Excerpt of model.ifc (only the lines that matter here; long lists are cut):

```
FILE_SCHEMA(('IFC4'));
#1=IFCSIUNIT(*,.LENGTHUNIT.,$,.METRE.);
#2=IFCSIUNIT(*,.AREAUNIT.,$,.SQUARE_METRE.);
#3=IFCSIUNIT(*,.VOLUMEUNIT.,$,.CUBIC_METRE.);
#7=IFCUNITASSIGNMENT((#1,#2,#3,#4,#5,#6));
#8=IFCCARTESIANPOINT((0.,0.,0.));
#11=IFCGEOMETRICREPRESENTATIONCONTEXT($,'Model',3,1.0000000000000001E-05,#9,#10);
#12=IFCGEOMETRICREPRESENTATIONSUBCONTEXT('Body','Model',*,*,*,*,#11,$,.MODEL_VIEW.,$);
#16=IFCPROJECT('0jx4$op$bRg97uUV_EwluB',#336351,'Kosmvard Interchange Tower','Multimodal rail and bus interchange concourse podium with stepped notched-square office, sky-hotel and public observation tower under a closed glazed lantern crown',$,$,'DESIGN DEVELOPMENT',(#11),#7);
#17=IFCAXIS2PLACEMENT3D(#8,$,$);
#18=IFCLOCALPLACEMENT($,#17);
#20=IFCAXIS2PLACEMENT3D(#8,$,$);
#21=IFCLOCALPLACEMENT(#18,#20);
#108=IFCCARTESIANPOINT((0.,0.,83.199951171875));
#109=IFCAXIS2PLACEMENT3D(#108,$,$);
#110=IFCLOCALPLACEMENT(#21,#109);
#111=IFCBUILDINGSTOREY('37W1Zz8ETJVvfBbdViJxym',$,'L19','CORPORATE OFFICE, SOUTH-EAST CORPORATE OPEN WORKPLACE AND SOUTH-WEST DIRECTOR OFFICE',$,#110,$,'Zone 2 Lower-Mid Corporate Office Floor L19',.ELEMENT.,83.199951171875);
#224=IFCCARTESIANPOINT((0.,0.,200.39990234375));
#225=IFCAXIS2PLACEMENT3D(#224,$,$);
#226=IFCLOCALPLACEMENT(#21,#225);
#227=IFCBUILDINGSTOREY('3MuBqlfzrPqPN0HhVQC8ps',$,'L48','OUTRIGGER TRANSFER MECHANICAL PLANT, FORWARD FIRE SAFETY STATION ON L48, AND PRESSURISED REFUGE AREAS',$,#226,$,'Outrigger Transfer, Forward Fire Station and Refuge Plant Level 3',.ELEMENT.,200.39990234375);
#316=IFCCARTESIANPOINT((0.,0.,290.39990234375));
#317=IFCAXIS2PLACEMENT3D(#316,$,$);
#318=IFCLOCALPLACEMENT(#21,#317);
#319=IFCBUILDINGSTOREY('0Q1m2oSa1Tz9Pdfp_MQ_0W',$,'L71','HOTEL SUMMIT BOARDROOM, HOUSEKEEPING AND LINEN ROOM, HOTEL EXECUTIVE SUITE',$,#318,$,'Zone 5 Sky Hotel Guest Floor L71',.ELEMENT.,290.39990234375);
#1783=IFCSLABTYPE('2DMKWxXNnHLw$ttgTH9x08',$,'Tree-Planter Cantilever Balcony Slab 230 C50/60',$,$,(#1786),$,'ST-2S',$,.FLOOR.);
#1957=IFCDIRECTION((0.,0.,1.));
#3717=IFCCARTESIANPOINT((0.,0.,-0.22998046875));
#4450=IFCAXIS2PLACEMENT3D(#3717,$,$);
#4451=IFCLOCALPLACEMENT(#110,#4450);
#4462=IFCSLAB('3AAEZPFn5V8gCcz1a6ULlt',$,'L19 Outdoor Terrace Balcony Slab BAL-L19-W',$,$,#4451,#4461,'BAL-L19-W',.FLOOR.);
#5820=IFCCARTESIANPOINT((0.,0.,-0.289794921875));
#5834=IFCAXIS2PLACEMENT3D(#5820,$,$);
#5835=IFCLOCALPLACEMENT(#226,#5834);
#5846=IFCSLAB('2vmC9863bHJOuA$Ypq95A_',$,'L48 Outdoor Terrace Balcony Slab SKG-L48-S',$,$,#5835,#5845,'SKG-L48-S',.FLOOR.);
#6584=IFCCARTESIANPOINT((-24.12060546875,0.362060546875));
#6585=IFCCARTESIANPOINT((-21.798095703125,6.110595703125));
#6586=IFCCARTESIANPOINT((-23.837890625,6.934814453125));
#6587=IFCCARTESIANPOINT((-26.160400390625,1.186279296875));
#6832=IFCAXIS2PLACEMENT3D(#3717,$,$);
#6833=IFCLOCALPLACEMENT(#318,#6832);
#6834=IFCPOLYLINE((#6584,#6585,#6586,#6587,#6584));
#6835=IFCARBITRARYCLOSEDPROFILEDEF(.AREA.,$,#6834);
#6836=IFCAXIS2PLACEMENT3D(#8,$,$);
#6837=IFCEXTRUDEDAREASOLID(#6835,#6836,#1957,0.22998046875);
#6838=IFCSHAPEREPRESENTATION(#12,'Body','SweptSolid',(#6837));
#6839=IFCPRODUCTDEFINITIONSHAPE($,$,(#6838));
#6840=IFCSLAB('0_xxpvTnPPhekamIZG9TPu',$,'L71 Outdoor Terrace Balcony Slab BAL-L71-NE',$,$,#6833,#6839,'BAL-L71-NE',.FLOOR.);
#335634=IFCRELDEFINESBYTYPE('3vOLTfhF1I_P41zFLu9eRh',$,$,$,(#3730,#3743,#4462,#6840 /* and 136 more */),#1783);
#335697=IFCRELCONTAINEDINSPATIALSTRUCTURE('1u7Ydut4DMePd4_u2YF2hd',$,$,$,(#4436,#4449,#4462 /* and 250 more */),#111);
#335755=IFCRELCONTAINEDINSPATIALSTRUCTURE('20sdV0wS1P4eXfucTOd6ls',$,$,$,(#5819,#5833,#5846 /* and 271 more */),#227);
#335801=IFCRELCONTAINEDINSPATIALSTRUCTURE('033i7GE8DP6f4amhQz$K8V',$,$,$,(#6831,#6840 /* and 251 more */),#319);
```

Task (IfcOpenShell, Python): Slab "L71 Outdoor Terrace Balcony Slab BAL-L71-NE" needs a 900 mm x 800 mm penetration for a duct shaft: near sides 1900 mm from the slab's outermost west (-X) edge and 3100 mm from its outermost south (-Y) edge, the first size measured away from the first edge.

```python
import numpy as np
import ifcopenshell
import ifcopenshell.api.feature
import ifcopenshell.api.geometry
import ifcopenshell.api.root
import ifcopenshell.geom
import ifcopenshell.util.placement
import ifcopenshell.util.representation
import ifcopenshell.util.shape
import ifcopenshell.util.unit

model = ifcopenshell.open("model.ifc")
unit_scale = ifcopenshell.util.unit.calculate_unit_scale(model)
settings = ifcopenshell.geom.settings()


def volume(element):
    """Net volume in cubic metres, openings subtracted."""
    shape = ifcopenshell.geom.create_shape(settings, element)
    return ifcopenshell.util.shape.get_volume(shape.geometry)


slab = model.by_guid("0_xxpvTnPPhekamIZG9TPu")
before = volume(slab)

# Extent in the slab's own axes, in metres. The edges named are its -X and -Y sides.
slab_shape = ifcopenshell.geom.create_shape(settings, slab)
vertices = ifcopenshell.util.shape.get_vertices(slab_shape.geometry)
x_min, y_min, bottom = vertices.min(axis=0)
top = vertices[:, 2].max()

opening = ifcopenshell.api.root.create_entity(model, ifc_class="IfcOpeningElement", name="Duct shaft opening", predefined_type="OPENING")
context = ifcopenshell.util.representation.get_context(model, "Model", "Body", "MODEL_VIEW")
width, depth = 0.9, 0.8
outline = [(0.0, 0.0), (width, 0.0), (width, depth), (0.0, depth), (0.0, 0.0)]
# Overshoot both faces by 50 mm so the cut is clean.
shape = ifcopenshell.api.geometry.add_slab_representation(
    model, context=context, depth=top - bottom + 0.1, polyline=outline
)
ifcopenshell.api.geometry.assign_representation(model, product=opening, representation=shape)

matrix = ifcopenshell.util.placement.get_local_placement(slab.ObjectPlacement)
matrix[:, 3] = matrix @ np.append(np.array([x_min + 1.9, y_min + 3.1, bottom - 0.05]) / unit_scale, 1.0)
ifcopenshell.api.geometry.edit_object_placement(model, product=opening, matrix=matrix, is_si=False)
ifcopenshell.api.feature.add_feature(model, feature=opening, element=slab)

after = volume(slab)

print(f"slab volume {before:.3f} -> {after:.3f} m3")

model.write("model_rev.ifc")
```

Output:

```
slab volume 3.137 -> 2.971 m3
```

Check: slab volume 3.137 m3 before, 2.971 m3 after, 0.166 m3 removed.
